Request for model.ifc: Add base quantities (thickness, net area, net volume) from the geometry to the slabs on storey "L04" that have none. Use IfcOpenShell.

First a look at what the model holds.

```python
import ifcopenshell
import ifcopenshell.util.element
import ifcopenshell.util.unit

model = ifcopenshell.open("model.ifc")
print(model.schema)
for unit_type in ("LENGTHUNIT", "AREAUNIT", "VOLUMEUNIT"):
    print(unit_type, ifcopenshell.util.unit.calculate_unit_scale(model, unit_type))
storey = next(s for s in model.by_type("IfcBuildingStorey") if s.Name == "L04")
slabs = [e for e in ifcopenshell.util.element.get_decomposition(storey) if e.is_a("IfcSlab")]
for e in sorted(slabs, key=lambda e: e.id()):
    print(e.id(), e.is_a(), e.Name, list(ifcopenshell.util.element.get_psets(e, qtos_only=True)), sep=" | ")
```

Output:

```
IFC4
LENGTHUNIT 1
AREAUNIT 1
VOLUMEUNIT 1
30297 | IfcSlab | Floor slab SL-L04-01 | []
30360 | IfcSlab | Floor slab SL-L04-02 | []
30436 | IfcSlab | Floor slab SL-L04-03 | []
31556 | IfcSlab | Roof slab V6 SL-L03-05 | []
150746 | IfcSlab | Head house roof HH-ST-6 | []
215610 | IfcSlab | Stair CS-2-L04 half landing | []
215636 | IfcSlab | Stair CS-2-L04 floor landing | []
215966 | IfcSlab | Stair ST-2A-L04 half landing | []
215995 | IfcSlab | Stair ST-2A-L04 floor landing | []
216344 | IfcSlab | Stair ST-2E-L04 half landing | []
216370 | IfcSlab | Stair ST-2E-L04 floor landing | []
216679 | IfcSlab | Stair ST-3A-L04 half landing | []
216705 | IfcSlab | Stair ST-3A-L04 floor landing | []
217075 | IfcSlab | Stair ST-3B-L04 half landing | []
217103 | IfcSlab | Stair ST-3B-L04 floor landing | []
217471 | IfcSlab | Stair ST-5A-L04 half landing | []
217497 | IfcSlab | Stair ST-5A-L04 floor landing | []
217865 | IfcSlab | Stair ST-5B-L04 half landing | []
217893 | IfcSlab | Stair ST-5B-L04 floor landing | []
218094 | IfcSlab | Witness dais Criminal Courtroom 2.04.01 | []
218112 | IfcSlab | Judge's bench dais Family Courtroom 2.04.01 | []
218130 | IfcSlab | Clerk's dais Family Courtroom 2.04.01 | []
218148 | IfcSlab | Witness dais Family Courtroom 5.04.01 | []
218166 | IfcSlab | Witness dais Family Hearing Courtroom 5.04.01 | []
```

```python
import ifcopenshell
import ifcopenshell.api.pset
import ifcopenshell.geom
import ifcopenshell.util.element
import ifcopenshell.util.shape
import ifcopenshell.util.unit

model = ifcopenshell.open("model.ifc")
unit_scale = ifcopenshell.util.unit.calculate_unit_scale(model)
area_scale = ifcopenshell.util.unit.calculate_unit_scale(model, "AREAUNIT")
volume_scale = ifcopenshell.util.unit.calculate_unit_scale(model, "VOLUMEUNIT")
settings = ifcopenshell.geom.settings()

storey = next(s for s in model.by_type("IfcBuildingStorey") if s.Name == "L04")
slabs = [e for e in ifcopenshell.util.element.get_decomposition(storey) if e.is_a("IfcSlab")]

for e in sorted(slabs, key=lambda e: e.id()):
    if ifcopenshell.util.element.get_psets(e, qtos_only=True, should_inherit=False):
        continue
    # Geometry comes back in metres, in the element's own axes.
    shape = ifcopenshell.geom.create_shape(settings, e)
    values = {
        "Width": ifcopenshell.util.shape.get_z(shape.geometry) / unit_scale,
        "NetArea": ifcopenshell.util.shape.get_footprint_area(shape.geometry) / area_scale,
        "NetVolume": ifcopenshell.util.shape.get_volume(shape.geometry) / volume_scale,
    }
    qto = ifcopenshell.api.pset.add_qto(model, product=e, name="Qto_SlabBaseQuantities")
    ifcopenshell.api.pset.edit_qto(model, qto=qto, properties=values)
    print(e.id(), {k: round(v, 3) for k, v in values.items()})

model.write("model_rev.ifc")
```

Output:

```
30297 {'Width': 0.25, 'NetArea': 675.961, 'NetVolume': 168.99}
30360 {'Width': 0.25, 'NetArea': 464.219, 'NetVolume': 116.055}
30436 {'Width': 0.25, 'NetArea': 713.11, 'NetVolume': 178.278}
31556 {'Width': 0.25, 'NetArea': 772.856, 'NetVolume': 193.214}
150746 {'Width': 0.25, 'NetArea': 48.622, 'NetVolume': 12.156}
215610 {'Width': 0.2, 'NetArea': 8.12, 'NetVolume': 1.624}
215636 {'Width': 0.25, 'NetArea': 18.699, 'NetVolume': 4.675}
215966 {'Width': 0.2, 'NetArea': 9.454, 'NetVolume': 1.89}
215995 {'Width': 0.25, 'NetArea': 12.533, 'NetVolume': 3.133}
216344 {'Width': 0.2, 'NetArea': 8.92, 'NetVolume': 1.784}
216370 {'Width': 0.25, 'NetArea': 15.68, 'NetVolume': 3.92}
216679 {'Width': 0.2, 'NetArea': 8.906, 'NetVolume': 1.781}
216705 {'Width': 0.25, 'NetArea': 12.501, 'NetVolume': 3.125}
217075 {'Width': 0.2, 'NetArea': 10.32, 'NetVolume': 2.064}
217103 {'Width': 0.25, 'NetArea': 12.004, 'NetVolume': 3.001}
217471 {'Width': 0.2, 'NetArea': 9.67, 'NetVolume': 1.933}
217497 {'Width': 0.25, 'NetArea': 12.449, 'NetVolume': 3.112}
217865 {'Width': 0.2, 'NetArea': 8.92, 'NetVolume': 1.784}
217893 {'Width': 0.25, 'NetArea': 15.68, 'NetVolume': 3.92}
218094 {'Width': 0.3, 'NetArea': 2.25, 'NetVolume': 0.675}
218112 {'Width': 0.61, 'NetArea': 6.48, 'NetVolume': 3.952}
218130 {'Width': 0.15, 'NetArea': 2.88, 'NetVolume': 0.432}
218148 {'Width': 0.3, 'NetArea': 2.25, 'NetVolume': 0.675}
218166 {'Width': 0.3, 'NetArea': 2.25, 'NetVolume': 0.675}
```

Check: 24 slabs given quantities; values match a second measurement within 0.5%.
